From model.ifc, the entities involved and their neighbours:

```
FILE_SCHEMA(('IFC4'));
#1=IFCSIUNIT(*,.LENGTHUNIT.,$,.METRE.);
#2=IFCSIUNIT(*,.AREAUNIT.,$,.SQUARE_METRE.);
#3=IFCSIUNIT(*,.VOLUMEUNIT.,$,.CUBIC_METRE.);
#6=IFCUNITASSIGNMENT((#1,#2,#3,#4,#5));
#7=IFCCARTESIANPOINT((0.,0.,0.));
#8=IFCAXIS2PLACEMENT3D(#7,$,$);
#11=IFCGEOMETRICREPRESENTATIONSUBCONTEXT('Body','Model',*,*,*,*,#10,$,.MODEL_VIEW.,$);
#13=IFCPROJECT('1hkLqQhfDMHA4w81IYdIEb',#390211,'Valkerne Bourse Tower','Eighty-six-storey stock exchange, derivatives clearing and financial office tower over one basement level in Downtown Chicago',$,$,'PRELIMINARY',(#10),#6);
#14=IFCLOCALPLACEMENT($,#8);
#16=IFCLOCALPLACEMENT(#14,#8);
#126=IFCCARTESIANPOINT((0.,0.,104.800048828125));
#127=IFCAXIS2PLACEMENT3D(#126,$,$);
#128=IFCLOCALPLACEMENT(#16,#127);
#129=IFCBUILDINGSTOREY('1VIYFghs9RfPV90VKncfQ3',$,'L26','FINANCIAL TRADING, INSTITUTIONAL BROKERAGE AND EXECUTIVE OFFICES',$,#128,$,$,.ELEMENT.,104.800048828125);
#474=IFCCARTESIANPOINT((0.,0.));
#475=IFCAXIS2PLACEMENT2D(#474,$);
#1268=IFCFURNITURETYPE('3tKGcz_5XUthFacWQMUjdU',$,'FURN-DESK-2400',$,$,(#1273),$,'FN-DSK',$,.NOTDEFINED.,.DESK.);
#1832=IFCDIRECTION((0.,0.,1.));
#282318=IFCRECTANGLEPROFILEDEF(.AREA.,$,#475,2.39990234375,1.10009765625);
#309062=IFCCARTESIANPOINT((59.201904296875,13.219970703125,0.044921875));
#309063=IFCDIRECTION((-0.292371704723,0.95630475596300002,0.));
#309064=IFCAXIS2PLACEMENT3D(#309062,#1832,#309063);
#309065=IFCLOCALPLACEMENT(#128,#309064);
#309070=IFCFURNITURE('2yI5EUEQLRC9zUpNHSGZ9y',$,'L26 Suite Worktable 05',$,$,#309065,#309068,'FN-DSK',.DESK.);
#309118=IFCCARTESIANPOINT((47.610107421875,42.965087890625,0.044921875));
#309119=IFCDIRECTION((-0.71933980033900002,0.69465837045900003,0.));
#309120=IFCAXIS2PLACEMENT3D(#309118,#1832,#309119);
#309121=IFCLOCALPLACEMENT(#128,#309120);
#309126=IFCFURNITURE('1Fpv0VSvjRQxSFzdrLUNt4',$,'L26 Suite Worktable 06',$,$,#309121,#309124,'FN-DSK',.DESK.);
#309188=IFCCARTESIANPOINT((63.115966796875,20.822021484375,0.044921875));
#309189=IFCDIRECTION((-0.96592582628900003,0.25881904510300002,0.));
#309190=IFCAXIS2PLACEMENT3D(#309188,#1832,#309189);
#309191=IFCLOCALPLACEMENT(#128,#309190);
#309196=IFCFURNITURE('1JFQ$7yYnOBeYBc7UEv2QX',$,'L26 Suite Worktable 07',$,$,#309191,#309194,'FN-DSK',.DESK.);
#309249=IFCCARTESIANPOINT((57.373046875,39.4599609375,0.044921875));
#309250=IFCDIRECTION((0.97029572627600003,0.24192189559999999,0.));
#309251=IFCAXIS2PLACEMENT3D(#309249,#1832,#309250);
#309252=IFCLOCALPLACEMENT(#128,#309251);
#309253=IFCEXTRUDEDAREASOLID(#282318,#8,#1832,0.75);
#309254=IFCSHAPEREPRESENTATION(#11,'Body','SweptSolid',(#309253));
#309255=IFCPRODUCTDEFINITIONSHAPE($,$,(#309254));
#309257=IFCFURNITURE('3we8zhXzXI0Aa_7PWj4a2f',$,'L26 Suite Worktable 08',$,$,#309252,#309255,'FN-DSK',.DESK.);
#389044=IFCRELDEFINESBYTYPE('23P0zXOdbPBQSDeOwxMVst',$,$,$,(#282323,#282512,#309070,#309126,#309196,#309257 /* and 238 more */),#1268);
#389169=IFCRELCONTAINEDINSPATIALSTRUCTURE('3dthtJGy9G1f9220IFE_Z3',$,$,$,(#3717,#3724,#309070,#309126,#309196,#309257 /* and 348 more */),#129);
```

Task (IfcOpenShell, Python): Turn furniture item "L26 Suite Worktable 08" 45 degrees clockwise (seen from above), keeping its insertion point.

```python
import ifcopenshell
import ifcopenshell.api.geometry
import ifcopenshell.util.placement

model = ifcopenshell.open("model.ifc")

item = model.by_guid("3we8zhXzXI0Aa_7PWj4a2f")
matrix = ifcopenshell.util.placement.get_local_placement(item.ObjectPlacement)
matrix = matrix @ ifcopenshell.util.placement.rotation(-45, "Z")
ifcopenshell.api.geometry.edit_object_placement(model, product=item, matrix=matrix, is_si=False)

print(ifcopenshell.util.placement.get_local_placement(item.ObjectPlacement).round(3) + 0.0)

model.write("model_updated.ifc")
```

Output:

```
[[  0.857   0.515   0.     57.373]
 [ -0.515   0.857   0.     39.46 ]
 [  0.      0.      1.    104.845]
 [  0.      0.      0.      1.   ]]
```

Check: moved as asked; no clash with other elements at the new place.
